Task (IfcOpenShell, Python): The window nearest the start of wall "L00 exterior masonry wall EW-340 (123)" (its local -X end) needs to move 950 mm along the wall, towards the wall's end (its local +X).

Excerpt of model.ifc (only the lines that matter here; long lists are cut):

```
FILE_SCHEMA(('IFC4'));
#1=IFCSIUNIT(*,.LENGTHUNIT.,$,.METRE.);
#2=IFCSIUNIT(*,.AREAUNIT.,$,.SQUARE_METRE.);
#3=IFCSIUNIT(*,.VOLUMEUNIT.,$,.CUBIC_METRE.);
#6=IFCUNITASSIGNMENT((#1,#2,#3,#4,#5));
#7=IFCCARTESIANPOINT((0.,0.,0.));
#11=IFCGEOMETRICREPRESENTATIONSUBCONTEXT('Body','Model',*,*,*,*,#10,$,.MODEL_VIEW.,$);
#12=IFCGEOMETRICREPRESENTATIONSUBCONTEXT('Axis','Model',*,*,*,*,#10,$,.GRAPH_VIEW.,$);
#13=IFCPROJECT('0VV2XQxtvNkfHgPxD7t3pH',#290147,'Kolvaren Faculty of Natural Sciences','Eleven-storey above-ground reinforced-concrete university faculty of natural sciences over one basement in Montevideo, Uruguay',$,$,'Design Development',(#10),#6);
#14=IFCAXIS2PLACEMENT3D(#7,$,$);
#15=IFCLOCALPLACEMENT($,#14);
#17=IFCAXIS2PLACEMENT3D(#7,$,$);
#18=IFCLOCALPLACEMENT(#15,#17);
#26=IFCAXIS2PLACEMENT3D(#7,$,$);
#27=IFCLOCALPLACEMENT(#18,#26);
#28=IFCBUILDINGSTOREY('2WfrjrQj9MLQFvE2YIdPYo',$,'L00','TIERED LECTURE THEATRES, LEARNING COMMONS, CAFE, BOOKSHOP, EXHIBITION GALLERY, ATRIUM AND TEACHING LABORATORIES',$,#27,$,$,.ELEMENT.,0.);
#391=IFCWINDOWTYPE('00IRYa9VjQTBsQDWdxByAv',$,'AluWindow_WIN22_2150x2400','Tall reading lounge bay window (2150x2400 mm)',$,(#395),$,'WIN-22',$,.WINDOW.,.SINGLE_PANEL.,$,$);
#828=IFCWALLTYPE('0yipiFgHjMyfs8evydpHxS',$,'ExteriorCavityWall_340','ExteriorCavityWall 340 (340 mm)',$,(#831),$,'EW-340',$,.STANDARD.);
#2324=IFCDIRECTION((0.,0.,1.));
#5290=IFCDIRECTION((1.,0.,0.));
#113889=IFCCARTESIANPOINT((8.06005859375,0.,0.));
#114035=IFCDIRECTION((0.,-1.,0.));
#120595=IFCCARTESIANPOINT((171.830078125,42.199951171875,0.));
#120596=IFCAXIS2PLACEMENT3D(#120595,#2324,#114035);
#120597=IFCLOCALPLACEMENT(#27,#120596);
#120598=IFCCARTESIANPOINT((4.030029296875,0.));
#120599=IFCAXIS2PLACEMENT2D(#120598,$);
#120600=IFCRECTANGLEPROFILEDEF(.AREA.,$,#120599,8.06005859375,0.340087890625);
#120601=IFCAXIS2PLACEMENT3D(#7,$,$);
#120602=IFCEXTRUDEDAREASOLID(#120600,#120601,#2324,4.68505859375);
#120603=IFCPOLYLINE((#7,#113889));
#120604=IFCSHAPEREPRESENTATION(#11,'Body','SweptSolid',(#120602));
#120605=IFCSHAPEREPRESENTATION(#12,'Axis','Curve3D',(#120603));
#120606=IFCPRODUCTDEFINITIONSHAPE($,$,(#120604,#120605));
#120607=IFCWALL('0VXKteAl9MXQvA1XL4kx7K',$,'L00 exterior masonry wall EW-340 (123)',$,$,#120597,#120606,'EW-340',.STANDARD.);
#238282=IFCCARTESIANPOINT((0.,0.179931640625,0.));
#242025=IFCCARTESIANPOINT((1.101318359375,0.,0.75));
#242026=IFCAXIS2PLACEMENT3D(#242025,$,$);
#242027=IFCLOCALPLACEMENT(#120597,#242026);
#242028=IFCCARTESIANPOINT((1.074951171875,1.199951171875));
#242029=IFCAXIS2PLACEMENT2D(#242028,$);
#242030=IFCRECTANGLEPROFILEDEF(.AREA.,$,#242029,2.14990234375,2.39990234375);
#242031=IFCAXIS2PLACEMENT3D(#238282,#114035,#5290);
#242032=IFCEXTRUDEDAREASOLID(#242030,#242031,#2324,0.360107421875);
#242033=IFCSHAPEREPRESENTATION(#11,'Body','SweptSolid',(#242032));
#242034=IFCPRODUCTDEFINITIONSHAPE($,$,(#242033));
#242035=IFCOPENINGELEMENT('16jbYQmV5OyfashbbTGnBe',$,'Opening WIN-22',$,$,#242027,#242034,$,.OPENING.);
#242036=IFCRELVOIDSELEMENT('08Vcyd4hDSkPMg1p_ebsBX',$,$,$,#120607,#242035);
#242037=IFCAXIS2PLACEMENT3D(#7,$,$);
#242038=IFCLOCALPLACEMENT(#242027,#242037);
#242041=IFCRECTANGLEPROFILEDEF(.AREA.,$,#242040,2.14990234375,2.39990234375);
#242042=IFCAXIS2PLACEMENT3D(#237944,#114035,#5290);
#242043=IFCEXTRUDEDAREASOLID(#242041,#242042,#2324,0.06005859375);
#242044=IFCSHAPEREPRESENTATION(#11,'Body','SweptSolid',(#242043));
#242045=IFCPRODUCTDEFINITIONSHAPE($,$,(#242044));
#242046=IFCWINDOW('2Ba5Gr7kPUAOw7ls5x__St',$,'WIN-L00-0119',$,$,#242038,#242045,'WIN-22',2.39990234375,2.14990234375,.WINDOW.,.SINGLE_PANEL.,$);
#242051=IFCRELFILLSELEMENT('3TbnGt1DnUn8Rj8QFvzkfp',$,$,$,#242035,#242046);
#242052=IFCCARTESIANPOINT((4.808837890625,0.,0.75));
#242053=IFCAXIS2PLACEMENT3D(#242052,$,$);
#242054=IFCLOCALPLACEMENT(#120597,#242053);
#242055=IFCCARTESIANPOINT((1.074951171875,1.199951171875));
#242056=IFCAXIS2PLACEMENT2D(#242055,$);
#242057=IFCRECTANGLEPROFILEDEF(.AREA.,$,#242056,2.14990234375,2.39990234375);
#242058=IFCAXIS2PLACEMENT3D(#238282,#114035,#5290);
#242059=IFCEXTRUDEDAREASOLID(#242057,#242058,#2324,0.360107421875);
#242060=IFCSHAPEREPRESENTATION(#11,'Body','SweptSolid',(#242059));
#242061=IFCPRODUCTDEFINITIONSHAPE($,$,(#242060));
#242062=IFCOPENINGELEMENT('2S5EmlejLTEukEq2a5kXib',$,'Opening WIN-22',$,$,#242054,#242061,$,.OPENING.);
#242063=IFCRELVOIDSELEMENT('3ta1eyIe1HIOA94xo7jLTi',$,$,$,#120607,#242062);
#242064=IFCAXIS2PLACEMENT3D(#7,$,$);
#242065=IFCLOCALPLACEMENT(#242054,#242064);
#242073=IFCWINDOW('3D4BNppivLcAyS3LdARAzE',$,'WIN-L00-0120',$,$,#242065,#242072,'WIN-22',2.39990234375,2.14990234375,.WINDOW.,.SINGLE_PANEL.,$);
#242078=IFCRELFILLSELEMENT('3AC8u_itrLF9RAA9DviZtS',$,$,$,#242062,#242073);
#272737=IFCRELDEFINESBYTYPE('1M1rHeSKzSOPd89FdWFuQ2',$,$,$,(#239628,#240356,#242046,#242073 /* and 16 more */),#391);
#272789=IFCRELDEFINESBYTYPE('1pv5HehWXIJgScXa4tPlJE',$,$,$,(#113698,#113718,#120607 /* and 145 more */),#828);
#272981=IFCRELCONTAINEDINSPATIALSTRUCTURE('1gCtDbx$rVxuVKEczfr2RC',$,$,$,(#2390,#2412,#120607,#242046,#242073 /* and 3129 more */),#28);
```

```python
import ifcopenshell
import ifcopenshell.api.geometry
import ifcopenshell.util.placement
import ifcopenshell.util.unit

model = ifcopenshell.open("model.ifc")
unit_scale = ifcopenshell.util.unit.calculate_unit_scale(model)

window = model.by_id(242046)
opening = window.FillsVoids[0].RelatingOpeningElement
wall = opening.VoidsElements[0].RelatingBuildingElement

wall_matrix = ifcopenshell.util.placement.get_local_placement(wall.ObjectPlacement)
shift = wall_matrix[:3, 0] * 0.95 / unit_scale
before = ifcopenshell.util.placement.get_local_placement(window.ObjectPlacement)[:3, 3].copy()

# The window is placed relative to its opening, so it follows when the opening moves.
matrix = ifcopenshell.util.placement.get_local_placement(opening.ObjectPlacement)
matrix[:3, 3] += shift
ifcopenshell.api.geometry.edit_object_placement(
    model, product=opening, matrix=matrix, is_si=False, should_transform_children=True
)

after = ifcopenshell.util.placement.get_local_placement(window.ObjectPlacement)[:3, 3]
print("window moved by", (after - before).round(3) + 0.0)

model.write("model_updated.ifc")
```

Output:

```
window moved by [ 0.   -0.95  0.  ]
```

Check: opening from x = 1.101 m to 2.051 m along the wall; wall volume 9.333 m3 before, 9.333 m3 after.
